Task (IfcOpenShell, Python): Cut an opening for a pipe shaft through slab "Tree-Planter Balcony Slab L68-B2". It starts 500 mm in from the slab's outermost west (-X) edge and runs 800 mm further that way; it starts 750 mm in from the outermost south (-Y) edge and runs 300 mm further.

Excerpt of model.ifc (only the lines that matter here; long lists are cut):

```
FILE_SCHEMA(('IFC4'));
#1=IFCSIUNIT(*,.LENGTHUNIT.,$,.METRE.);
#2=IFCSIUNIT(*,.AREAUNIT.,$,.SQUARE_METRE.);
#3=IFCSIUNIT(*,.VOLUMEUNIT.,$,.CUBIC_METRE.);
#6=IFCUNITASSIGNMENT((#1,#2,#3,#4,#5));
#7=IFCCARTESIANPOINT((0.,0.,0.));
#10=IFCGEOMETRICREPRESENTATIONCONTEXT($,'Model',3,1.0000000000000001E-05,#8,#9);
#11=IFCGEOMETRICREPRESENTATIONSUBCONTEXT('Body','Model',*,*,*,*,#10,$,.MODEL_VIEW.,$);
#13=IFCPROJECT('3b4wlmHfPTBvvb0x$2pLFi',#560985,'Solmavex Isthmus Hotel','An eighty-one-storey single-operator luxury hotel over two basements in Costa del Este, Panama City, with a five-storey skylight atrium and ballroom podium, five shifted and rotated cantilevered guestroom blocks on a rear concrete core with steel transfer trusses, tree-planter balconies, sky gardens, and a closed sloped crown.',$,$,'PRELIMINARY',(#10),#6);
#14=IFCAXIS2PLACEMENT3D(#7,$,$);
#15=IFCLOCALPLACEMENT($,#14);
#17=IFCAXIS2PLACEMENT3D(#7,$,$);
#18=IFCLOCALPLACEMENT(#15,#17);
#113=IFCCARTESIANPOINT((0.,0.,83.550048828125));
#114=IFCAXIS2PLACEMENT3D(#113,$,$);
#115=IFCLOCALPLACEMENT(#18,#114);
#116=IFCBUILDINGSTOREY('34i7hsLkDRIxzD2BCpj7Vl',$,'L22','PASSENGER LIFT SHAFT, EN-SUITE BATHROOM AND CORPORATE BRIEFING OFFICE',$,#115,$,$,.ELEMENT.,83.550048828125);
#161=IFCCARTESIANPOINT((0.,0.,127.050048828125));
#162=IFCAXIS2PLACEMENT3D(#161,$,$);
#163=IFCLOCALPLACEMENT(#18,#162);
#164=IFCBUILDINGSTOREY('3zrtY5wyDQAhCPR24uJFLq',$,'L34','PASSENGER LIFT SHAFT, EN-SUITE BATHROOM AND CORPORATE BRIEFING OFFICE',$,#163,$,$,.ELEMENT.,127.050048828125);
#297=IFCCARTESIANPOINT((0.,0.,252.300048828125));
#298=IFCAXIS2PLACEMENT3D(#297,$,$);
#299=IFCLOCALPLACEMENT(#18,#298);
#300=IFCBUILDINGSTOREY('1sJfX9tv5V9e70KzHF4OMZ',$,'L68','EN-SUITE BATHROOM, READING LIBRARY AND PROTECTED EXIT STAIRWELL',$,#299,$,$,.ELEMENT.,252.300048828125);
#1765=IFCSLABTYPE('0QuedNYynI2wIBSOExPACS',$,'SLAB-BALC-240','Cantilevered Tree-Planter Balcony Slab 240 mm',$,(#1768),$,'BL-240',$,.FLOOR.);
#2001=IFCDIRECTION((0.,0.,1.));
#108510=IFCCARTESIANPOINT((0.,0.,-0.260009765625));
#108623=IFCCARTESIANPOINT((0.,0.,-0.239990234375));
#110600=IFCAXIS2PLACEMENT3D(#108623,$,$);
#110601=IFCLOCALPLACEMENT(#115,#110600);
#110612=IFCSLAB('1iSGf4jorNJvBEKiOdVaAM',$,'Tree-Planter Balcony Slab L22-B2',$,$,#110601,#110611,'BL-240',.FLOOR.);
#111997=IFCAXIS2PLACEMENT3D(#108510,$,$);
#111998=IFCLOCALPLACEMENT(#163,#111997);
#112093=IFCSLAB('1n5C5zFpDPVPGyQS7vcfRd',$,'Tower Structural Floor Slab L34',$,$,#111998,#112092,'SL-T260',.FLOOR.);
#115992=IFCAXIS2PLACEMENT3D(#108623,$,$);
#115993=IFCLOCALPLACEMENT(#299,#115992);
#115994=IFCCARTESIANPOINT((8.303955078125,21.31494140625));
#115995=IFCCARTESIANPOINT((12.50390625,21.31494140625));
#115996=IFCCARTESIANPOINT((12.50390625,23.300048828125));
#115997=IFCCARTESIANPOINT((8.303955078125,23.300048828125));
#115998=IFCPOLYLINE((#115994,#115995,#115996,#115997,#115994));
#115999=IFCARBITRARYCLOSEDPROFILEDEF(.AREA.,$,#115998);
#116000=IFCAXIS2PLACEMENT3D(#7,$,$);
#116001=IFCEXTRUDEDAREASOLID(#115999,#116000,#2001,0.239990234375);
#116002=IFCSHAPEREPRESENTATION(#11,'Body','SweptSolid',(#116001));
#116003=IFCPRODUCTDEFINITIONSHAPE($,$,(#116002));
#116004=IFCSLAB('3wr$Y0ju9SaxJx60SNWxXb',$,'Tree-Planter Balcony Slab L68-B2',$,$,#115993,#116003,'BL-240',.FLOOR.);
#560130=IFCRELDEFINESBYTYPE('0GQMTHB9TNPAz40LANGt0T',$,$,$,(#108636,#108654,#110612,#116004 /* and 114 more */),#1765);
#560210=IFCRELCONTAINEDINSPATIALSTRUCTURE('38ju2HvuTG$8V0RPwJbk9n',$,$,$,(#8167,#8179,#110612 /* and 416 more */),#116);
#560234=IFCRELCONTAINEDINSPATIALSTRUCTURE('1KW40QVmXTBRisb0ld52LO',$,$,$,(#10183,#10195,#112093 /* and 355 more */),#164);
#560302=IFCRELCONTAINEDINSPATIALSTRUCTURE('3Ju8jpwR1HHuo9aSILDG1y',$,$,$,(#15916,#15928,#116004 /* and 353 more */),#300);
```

```python
import numpy as np
import ifcopenshell
import ifcopenshell.api.feature
import ifcopenshell.api.geometry
import ifcopenshell.api.root
import ifcopenshell.geom
import ifcopenshell.util.placement
import ifcopenshell.util.representation
import ifcopenshell.util.shape
import ifcopenshell.util.unit

model = ifcopenshell.open("model.ifc")
unit_scale = ifcopenshell.util.unit.calculate_unit_scale(model)
settings = ifcopenshell.geom.settings()


def volume(element):
    """Net volume in cubic metres, openings subtracted."""
    shape = ifcopenshell.geom.create_shape(settings, element)
    return ifcopenshell.util.shape.get_volume(shape.geometry)


slab = model.by_guid("3wr$Y0ju9SaxJx60SNWxXb")
before = volume(slab)

# Extent in the slab's own axes, in metres. The edges named are its -X and -Y sides.
slab_shape = ifcopenshell.geom.create_shape(settings, slab)
vertices = ifcopenshell.util.shape.get_vertices(slab_shape.geometry)
x_min, y_min, bottom = vertices.min(axis=0)
top = vertices[:, 2].max()

opening = ifcopenshell.api.root.create_entity(model, ifc_class="IfcOpeningElement", name="Pipe shaft opening", predefined_type="OPENING")
context = ifcopenshell.util.representation.get_context(model, "Model", "Body", "MODEL_VIEW")
width, depth = 0.8, 0.3
outline = [(0.0, 0.0), (width, 0.0), (width, depth), (0.0, depth), (0.0, 0.0)]
# Overshoot both faces by 50 mm so the cut is clean.
shape = ifcopenshell.api.geometry.add_slab_representation(
    model, context=context, depth=top - bottom + 0.1, polyline=outline
)
ifcopenshell.api.geometry.assign_representation(model, product=opening, representation=shape)

matrix = ifcopenshell.util.placement.get_local_placement(slab.ObjectPlacement)
matrix[:, 3] = matrix @ np.append(np.array([x_min + 0.5, y_min + 0.75, bottom - 0.05]) / unit_scale, 1.0)
ifcopenshell.api.geometry.edit_object_placement(model, product=opening, matrix=matrix, is_si=False)
ifcopenshell.api.feature.add_feature(model, feature=opening, element=slab)

after = volume(slab)

print(f"slab volume {before:.3f} -> {after:.3f} m3")

model.write("model_edited.ifc")
```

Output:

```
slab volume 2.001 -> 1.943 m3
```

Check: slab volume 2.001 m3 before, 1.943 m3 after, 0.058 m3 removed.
